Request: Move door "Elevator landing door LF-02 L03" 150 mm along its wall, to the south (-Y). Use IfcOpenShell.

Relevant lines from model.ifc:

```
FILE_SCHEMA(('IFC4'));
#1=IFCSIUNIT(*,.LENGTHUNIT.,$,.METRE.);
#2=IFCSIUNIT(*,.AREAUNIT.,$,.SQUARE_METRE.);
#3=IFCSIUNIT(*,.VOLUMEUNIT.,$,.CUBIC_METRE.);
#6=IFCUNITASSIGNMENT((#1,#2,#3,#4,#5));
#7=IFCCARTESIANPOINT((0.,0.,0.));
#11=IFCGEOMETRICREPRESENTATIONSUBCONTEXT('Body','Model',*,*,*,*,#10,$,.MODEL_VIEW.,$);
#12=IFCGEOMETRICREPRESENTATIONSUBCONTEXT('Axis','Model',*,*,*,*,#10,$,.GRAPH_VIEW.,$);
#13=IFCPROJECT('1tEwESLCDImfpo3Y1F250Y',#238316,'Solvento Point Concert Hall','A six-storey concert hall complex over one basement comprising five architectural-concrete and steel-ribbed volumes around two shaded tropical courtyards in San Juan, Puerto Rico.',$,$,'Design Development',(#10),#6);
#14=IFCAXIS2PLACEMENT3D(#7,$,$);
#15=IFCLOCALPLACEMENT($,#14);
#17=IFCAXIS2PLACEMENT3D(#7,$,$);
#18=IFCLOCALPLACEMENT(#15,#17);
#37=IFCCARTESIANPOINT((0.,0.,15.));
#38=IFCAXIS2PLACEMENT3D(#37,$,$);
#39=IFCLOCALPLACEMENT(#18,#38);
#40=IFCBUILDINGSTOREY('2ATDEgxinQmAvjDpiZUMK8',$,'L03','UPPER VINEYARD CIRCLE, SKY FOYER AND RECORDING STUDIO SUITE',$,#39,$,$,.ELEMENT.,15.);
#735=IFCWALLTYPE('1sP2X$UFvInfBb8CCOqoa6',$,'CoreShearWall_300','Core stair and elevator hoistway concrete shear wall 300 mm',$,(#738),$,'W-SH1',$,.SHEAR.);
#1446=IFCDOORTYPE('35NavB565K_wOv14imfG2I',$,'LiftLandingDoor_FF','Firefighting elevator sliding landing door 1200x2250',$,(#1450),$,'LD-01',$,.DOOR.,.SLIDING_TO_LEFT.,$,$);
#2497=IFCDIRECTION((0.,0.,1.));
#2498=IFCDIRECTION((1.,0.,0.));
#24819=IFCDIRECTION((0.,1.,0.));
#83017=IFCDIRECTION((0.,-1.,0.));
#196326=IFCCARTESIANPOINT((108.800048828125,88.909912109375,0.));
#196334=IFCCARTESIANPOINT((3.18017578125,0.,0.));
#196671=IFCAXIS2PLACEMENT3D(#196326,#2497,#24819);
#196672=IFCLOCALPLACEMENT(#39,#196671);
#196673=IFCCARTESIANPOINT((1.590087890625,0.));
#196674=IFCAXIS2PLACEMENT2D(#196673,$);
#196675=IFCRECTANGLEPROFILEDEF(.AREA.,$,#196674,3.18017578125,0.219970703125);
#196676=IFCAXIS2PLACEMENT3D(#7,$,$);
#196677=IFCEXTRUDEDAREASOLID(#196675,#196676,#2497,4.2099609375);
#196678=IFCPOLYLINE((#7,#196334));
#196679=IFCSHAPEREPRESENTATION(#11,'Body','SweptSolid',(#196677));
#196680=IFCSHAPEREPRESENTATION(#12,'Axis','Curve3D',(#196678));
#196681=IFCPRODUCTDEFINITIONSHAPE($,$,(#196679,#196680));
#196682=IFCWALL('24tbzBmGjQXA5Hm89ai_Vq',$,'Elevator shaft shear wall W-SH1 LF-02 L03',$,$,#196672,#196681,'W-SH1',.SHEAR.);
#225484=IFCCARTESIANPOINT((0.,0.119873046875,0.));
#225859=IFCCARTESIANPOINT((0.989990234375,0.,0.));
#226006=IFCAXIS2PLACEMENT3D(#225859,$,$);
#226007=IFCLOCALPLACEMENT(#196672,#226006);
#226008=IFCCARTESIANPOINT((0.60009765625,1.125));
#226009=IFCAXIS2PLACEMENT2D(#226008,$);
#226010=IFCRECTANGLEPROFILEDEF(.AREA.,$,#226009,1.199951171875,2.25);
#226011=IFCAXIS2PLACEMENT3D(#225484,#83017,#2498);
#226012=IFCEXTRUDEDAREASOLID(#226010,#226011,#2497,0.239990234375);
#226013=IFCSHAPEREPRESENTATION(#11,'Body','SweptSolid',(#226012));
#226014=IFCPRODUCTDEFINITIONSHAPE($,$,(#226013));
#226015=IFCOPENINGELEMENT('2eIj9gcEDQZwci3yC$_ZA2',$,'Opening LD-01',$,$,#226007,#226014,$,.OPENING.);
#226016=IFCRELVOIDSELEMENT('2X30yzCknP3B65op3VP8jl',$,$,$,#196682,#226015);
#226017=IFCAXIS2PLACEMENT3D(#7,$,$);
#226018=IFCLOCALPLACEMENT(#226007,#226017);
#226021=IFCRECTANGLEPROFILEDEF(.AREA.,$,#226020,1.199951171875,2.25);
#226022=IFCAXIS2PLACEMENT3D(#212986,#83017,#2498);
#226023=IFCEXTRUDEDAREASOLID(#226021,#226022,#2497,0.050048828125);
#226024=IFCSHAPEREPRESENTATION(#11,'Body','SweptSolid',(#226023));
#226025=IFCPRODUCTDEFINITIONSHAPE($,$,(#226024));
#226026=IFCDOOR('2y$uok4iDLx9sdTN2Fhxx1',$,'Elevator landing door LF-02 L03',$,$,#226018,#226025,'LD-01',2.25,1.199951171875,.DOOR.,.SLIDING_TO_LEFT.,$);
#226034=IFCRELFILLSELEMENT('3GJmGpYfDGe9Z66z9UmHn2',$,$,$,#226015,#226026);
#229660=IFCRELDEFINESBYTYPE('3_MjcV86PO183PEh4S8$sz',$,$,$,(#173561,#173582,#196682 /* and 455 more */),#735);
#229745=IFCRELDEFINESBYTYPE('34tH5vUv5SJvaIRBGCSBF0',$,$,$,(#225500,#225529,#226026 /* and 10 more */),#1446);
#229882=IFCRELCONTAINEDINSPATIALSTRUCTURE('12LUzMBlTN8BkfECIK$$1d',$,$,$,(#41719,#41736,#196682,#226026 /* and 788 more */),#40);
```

```python
import ifcopenshell
import ifcopenshell.api.geometry
import ifcopenshell.util.placement

model = ifcopenshell.open("model.ifc")

door = model.by_guid("2y$uok4iDLx9sdTN2Fhxx1")
opening = door.FillsVoids[0].RelatingOpeningElement
wall = opening.VoidsElements[0].RelatingBuildingElement

wall_matrix = ifcopenshell.util.placement.get_local_placement(wall.ObjectPlacement)
shift = wall_matrix[:3, 0] * -0.15
before = ifcopenshell.util.placement.get_local_placement(door.ObjectPlacement)[:3, 3].copy()

# The door is placed relative to its opening, so it follows when the opening moves.
matrix = ifcopenshell.util.placement.get_local_placement(opening.ObjectPlacement)
matrix[:3, 3] += shift
ifcopenshell.api.geometry.edit_object_placement(
    model, product=opening, matrix=matrix, is_si=False, should_transform_children=True
)

after = ifcopenshell.util.placement.get_local_placement(door.ObjectPlacement)[:3, 3]
print("door moved by", (after - before).round(3) + 0.0)

model.write("model_edited.ifc")
```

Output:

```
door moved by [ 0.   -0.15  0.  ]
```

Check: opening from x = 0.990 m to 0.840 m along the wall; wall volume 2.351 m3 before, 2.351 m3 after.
